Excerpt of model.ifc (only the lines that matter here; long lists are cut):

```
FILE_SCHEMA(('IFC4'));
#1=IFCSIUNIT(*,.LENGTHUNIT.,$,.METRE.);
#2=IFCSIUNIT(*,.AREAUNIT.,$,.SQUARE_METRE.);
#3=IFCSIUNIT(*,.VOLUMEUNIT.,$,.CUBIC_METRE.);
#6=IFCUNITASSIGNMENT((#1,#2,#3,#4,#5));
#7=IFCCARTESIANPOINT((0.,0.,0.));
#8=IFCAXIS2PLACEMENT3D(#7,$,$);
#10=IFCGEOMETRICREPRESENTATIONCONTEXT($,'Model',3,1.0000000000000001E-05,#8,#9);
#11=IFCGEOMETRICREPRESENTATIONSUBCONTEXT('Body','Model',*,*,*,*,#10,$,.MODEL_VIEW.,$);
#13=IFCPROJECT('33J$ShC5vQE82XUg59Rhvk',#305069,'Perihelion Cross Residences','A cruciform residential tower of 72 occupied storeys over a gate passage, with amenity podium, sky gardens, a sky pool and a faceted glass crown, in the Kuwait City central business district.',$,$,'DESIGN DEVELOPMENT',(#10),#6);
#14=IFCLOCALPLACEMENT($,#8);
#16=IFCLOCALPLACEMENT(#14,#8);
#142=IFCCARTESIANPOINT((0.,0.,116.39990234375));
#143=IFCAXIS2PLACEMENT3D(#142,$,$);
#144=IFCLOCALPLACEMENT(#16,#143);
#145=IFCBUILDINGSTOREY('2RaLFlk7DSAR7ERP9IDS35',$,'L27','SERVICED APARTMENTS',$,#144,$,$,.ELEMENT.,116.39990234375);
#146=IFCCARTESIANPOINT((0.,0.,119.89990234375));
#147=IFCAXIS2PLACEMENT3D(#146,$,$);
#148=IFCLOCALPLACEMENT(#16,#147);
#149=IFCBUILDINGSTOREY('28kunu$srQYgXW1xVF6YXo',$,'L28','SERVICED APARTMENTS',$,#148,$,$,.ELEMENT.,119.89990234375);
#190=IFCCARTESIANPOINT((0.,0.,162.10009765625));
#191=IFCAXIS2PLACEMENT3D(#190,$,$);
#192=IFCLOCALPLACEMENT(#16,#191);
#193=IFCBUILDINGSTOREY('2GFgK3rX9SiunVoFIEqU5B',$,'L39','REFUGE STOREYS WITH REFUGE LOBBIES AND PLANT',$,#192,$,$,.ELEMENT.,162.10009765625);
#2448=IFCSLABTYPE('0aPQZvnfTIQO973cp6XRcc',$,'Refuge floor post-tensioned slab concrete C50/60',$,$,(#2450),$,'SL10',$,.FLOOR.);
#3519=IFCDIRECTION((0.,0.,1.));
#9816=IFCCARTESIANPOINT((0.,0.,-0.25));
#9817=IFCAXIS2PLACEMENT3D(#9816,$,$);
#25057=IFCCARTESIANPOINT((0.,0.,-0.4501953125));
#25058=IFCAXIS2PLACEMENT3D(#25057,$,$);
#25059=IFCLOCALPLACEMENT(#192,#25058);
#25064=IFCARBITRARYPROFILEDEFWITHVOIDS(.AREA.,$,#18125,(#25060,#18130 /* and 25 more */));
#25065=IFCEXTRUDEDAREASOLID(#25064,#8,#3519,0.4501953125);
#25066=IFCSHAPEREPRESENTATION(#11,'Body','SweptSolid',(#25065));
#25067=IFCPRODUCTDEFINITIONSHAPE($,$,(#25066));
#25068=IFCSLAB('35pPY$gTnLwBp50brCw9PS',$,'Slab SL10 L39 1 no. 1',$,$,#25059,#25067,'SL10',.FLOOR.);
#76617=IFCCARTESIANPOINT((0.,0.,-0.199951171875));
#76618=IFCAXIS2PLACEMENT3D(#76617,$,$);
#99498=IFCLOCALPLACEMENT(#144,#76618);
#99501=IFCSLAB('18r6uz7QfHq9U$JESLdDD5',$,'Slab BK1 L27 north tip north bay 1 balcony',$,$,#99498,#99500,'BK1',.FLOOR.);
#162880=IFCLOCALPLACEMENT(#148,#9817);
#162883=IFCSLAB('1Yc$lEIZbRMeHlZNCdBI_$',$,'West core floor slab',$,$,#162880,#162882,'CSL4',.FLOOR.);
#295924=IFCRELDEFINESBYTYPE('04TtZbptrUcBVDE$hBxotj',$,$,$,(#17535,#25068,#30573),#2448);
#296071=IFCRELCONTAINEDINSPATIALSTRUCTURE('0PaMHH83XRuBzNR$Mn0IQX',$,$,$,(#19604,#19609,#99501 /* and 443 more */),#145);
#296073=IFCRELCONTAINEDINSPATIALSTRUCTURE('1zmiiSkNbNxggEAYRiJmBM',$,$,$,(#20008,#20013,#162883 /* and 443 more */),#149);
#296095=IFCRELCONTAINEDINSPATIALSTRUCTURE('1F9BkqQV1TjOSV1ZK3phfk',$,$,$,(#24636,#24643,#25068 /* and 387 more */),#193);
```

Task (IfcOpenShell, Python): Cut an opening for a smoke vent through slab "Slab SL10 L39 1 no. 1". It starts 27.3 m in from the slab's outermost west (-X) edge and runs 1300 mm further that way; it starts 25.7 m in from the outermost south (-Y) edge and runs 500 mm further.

```python
import numpy as np
import ifcopenshell
import ifcopenshell.api.feature
import ifcopenshell.api.geometry
import ifcopenshell.api.root
import ifcopenshell.geom
import ifcopenshell.util.placement
import ifcopenshell.util.representation
import ifcopenshell.util.shape
import ifcopenshell.util.unit

model = ifcopenshell.open("model.ifc")
unit_scale = ifcopenshell.util.unit.calculate_unit_scale(model)
settings = ifcopenshell.geom.settings()


def volume(element):
    """Net volume in cubic metres, openings subtracted."""
    shape = ifcopenshell.geom.create_shape(settings, element)
    return ifcopenshell.util.shape.get_volume(shape.geometry)


slab = model.by_id(25068)
before = volume(slab)

# Extent in the slab's own axes, in metres. The edges named are its -X and -Y sides.
slab_shape = ifcopenshell.geom.create_shape(settings, slab)
vertices = ifcopenshell.util.shape.get_vertices(slab_shape.geometry)
x_min, y_min, bottom = vertices.min(axis=0)
top = vertices[:, 2].max()

opening = ifcopenshell.api.root.create_entity(model, ifc_class="IfcOpeningElement", name="Smoke vent opening", predefined_type="OPENING")
context = ifcopenshell.util.representation.get_context(model, "Model", "Body", "MODEL_VIEW")
width, depth = 1.3, 0.5
outline = [(0.0, 0.0), (width, 0.0), (width, depth), (0.0, depth), (0.0, 0.0)]
# Overshoot both faces by 50 mm so the cut is clean.
shape = ifcopenshell.api.geometry.add_slab_representation(
    model, context=context, depth=top - bottom + 0.1, polyline=outline
)
ifcopenshell.api.geometry.assign_representation(model, product=opening, representation=shape)

matrix = ifcopenshell.util.placement.get_local_placement(slab.ObjectPlacement)
matrix[:, 3] = matrix @ np.append(np.array([x_min + 27.3, y_min + 25.7, bottom - 0.05]) / unit_scale, 1.0)
ifcopenshell.api.geometry.edit_object_placement(model, product=opening, matrix=matrix, is_si=False)
ifcopenshell.api.feature.add_feature(model, feature=opening, element=slab)

after = volume(slab)

print(f"slab volume {before:.3f} -> {after:.3f} m3")

model.write("model_updated.ifc")
```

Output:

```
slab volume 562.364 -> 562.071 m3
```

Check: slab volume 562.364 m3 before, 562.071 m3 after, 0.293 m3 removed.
